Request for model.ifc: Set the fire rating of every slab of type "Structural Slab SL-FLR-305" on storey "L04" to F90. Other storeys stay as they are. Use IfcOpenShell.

First a look at what the model holds.

```python
import ifcopenshell
import ifcopenshell.util.element

model = ifcopenshell.open("model.ifc")
print(model.schema)
storey = next(s for s in model.by_type("IfcBuildingStorey") if s.Name == "L04")
slabs = [e for e in ifcopenshell.util.element.get_decomposition(storey) if e.is_a("IfcSlab")]
seen = {}
for e in slabs:
    element_type = ifcopenshell.util.element.get_type(e)
    key = (element_type.Name if element_type != e and element_type else None, ifcopenshell.util.element.get_pset(e, "Pset_SlabCommon", "FireRating"))
    seen[key] = seen.get(key, 0) + 1
for (name, value), count in sorted(seen.items(), key=str):
    print(count, "x", name, "|", value)
```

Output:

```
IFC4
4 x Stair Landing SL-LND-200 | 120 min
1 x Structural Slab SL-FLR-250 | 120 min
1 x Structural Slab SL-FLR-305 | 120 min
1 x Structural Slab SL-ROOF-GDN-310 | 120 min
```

```python
import ifcopenshell
import ifcopenshell.api.pset
import ifcopenshell.util.element

model = ifcopenshell.open("model.ifc")

storey = next(s for s in model.by_type("IfcBuildingStorey") if s.Name == "L04")
slabs = [e for e in ifcopenshell.util.element.get_decomposition(storey) if e.is_a("IfcSlab")]

count = 0
for e in slabs:
    element_type = ifcopenshell.util.element.get_type(e)
    if element_type in (None, e) or element_type.Name != "Structural Slab SL-FLR-305":
        continue
    # add_pset returns the element's existing set when there is one.
    pset = ifcopenshell.api.pset.add_pset(model, product=e, name="Pset_SlabCommon")
    ifcopenshell.api.pset.edit_pset(model, pset=pset, properties={"FireRating": "F90"})
    count += 1

print(count, "slabs updated")

model.write("model_rev.ifc")
```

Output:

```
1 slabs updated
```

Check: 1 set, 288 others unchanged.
